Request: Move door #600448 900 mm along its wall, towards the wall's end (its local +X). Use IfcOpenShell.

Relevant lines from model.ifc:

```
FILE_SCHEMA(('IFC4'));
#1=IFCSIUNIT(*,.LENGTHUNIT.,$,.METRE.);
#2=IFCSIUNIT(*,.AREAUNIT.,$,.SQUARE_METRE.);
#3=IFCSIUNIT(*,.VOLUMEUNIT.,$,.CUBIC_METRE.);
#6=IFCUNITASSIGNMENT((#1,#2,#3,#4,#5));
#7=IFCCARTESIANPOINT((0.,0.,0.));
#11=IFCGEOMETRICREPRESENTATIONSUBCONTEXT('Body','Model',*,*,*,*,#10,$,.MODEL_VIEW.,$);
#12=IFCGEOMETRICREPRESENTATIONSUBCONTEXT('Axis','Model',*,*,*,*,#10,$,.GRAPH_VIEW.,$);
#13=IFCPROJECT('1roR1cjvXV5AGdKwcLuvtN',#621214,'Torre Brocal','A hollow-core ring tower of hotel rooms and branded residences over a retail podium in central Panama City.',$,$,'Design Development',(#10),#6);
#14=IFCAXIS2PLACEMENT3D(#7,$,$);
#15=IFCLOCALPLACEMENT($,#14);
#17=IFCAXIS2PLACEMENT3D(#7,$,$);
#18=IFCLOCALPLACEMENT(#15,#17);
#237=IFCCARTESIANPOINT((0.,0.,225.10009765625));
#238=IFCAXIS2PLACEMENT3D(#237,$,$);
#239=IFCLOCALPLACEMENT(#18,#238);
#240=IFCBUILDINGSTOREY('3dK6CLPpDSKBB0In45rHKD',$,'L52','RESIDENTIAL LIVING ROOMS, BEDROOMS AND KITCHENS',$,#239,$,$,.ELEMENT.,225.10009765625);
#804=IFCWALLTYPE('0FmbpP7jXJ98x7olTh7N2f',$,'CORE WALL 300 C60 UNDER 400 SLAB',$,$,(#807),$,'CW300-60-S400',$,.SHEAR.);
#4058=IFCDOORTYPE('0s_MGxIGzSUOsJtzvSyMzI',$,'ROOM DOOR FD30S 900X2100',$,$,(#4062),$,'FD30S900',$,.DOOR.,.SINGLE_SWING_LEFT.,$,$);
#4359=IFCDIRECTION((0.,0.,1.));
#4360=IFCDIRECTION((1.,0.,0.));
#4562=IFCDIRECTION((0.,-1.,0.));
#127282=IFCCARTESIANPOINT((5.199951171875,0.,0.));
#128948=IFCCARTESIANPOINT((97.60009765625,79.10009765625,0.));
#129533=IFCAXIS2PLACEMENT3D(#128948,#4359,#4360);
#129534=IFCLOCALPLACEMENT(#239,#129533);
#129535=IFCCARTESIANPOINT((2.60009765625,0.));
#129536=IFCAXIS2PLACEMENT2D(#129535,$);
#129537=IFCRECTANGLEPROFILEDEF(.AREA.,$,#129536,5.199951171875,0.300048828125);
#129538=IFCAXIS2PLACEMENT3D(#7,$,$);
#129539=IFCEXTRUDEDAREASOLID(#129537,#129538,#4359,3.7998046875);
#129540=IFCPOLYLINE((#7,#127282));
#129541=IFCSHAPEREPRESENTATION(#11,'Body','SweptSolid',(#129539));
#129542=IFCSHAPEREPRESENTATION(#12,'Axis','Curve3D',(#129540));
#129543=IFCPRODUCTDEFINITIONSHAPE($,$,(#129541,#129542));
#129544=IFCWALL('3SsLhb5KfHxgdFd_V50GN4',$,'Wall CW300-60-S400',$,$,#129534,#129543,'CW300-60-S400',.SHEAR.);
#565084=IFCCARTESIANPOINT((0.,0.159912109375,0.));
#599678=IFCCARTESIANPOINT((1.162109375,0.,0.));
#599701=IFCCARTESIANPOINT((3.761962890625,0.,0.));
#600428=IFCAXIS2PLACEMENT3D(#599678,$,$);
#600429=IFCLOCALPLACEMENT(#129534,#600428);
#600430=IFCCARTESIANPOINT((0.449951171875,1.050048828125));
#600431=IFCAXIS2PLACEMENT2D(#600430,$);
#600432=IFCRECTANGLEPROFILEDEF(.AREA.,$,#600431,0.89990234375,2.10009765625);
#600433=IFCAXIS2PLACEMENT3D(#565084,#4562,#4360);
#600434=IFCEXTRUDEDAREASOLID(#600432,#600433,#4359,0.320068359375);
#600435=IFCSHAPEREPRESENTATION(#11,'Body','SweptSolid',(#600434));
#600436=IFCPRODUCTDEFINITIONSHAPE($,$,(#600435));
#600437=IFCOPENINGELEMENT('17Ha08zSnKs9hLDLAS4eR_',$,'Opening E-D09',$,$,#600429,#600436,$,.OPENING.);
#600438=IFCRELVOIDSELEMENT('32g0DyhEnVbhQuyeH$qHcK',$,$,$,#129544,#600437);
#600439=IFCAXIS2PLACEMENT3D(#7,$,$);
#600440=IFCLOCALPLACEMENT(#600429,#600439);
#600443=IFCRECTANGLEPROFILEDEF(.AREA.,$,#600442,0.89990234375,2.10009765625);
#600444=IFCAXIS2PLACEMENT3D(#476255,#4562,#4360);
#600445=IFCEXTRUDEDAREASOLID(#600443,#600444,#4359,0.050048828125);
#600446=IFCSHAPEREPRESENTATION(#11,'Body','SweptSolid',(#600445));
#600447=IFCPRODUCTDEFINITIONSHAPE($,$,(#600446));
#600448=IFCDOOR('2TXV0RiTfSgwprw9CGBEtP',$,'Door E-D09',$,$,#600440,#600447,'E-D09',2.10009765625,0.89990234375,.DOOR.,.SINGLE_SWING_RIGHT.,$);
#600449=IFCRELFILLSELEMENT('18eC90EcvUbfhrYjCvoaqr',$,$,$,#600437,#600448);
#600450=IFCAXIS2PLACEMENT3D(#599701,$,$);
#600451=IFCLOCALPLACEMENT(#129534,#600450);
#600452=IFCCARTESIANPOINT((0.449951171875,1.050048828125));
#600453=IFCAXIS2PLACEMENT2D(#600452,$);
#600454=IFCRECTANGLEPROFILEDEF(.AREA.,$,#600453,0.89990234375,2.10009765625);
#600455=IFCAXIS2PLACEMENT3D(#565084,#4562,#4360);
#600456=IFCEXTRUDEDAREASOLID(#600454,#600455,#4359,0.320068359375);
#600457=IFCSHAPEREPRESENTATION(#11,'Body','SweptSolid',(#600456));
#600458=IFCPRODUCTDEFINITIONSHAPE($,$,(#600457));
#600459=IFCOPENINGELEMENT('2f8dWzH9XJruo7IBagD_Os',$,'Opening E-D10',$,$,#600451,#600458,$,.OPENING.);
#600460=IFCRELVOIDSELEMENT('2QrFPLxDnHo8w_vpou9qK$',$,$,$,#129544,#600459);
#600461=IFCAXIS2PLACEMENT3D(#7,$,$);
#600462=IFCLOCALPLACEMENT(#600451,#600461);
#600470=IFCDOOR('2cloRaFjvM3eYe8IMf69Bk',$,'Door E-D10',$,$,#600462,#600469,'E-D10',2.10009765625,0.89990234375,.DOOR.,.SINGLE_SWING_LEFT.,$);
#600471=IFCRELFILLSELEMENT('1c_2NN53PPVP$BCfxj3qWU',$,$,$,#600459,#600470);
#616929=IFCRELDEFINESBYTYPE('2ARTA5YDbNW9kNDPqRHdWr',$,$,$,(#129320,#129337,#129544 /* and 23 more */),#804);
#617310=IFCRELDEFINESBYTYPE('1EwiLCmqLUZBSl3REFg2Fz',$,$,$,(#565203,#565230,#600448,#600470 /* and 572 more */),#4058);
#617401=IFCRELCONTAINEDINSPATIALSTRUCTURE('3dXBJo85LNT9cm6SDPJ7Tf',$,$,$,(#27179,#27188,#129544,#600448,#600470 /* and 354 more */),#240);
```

```python
import ifcopenshell
import ifcopenshell.api.geometry
import ifcopenshell.util.placement
import ifcopenshell.util.unit

model = ifcopenshell.open("model.ifc")
unit_scale = ifcopenshell.util.unit.calculate_unit_scale(model)

door = model.by_guid("2TXV0RiTfSgwprw9CGBEtP")
opening = door.FillsVoids[0].RelatingOpeningElement
wall = opening.VoidsElements[0].RelatingBuildingElement

wall_matrix = ifcopenshell.util.placement.get_local_placement(wall.ObjectPlacement)
shift = wall_matrix[:3, 0] * 0.9 / unit_scale
before = ifcopenshell.util.placement.get_local_placement(door.ObjectPlacement)[:3, 3].copy()

# The door is placed relative to its opening, so it follows when the opening moves.
matrix = ifcopenshell.util.placement.get_local_placement(opening.ObjectPlacement)
matrix[:3, 3] += shift
ifcopenshell.api.geometry.edit_object_placement(
    model, product=opening, matrix=matrix, is_si=False, should_transform_children=True
)

after = ifcopenshell.util.placement.get_local_placement(door.ObjectPlacement)[:3, 3]
print("door moved by", (after - before).round(3) + 0.0)

model.write("model_v2.ifc")
```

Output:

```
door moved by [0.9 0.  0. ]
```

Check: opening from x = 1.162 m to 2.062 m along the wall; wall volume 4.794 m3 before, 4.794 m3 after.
